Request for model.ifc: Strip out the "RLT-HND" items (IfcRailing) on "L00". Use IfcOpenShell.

First a look at what the model holds.

```python
import ifcopenshell
import ifcopenshell.util.element

model = ifcopenshell.open("model.ifc")
print(model.schema)
storey = next(s for s in model.by_type("IfcBuildingStorey") if s.Name == "L00")
railings = [e for e in ifcopenshell.util.element.get_decomposition(storey) if e.is_a("IfcRailing")]
seen = {}
for e in railings:
    element_type = ifcopenshell.util.element.get_type(e)
    name = element_type.Name if element_type not in (None, e) else None
    seen[name] = seen.get(name, 0) + 1
for name, count in sorted(seen.items(), key=str):
    print(count, "x", name)
```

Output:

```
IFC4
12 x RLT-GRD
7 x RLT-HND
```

```python
import ifcopenshell
import ifcopenshell.api.root
import ifcopenshell.util.element

model = ifcopenshell.open("model.ifc")

storey = next(s for s in model.by_type("IfcBuildingStorey") if s.Name == "L00")
railings = [e for e in ifcopenshell.util.element.get_decomposition(storey) if e.is_a("IfcRailing")]
targets = [e for e in railings if (t := ifcopenshell.util.element.get_type(e)) not in (None, e) and t.Name == "RLT-HND"]

for e in targets:
    ifcopenshell.api.root.remove_product(model, product=e)
print(len(targets), "removed")

model.write("model-out.ifc")
```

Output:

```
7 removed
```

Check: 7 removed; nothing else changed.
